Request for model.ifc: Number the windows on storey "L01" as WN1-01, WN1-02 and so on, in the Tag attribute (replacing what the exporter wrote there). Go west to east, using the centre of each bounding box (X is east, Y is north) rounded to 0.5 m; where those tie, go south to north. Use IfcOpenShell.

First a look at what the model holds.

```python
import ifcopenshell
import ifcopenshell.util.element
import ifcopenshell.util.placement

model = ifcopenshell.open("model.ifc")
print(model.schema)
storey = next(s for s in model.by_type("IfcBuildingStorey") if s.Name == "L01")
windows = [e for e in ifcopenshell.util.element.get_decomposition(storey) if e.is_a("IfcWindow")]
for e in sorted(windows, key=lambda e: e.id()):
    origin = ifcopenshell.util.placement.get_local_placement(e.ObjectPlacement)[:3, 3]
    print(e.id(), e.Tag, e.Name, origin.round(2) + 0.0, sep=" | ")
```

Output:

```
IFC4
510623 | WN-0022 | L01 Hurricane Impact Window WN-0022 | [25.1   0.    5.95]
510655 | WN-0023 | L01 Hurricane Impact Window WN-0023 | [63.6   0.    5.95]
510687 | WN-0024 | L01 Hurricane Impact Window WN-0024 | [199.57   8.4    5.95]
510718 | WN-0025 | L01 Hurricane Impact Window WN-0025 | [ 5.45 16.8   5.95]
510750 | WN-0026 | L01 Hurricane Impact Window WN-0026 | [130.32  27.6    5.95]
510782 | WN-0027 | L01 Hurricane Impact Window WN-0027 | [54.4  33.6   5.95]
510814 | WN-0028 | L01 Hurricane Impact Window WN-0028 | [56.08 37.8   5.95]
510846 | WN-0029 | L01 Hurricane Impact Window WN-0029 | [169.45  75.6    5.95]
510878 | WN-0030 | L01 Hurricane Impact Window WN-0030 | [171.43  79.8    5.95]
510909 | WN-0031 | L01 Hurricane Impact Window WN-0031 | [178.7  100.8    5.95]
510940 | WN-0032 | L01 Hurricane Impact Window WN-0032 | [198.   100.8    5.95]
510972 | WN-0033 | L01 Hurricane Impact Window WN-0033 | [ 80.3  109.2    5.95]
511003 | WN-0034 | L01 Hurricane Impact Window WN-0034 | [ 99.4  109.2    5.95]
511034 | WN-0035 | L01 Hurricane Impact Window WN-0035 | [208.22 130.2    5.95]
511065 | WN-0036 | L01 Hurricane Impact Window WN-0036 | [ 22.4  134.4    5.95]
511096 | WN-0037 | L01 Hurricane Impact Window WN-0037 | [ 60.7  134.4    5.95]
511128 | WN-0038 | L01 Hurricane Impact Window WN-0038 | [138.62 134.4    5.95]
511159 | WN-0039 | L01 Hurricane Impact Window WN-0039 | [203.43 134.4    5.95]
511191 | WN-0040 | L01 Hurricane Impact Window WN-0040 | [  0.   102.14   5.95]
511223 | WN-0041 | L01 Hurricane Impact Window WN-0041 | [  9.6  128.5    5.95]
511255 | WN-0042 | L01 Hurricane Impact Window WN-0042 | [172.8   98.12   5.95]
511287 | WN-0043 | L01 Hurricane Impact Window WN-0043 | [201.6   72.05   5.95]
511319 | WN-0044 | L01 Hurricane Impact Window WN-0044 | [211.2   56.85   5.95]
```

```python
import ifcopenshell
import ifcopenshell.geom
import ifcopenshell.util.element
import ifcopenshell.util.shape

model = ifcopenshell.open("model.ifc")
settings = ifcopenshell.geom.settings()
settings.set("use-world-coords", True)


def centre(element):
    shape = ifcopenshell.geom.create_shape(settings, element)
    return ifcopenshell.util.shape.get_bbox_centroid(shape.geometry)


storey = next(s for s in model.by_type("IfcBuildingStorey") if s.Name == "L01")
windows = [e for e in ifcopenshell.util.element.get_decomposition(storey) if e.is_a("IfcWindow")]

# Insertion points can sit at a corner or the storey origin, so sort by the geometry (in metres).
centres = {e: centre(e) for e in windows}
windows.sort(key=lambda e: (round(centres[e][0] / 0.5), centres[e][1]))

for i, e in enumerate(windows, start=1):
    number = f"WN1-{i:02d}"
    e.Tag = number
    print(e.id(), number)

model.write("model_rev.ifc")
```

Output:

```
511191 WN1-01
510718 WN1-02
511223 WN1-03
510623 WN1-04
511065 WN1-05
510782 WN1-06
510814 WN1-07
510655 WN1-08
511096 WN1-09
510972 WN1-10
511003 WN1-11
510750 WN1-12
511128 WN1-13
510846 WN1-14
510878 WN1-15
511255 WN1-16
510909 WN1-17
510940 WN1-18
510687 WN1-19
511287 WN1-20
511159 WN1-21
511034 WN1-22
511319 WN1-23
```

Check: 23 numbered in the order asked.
